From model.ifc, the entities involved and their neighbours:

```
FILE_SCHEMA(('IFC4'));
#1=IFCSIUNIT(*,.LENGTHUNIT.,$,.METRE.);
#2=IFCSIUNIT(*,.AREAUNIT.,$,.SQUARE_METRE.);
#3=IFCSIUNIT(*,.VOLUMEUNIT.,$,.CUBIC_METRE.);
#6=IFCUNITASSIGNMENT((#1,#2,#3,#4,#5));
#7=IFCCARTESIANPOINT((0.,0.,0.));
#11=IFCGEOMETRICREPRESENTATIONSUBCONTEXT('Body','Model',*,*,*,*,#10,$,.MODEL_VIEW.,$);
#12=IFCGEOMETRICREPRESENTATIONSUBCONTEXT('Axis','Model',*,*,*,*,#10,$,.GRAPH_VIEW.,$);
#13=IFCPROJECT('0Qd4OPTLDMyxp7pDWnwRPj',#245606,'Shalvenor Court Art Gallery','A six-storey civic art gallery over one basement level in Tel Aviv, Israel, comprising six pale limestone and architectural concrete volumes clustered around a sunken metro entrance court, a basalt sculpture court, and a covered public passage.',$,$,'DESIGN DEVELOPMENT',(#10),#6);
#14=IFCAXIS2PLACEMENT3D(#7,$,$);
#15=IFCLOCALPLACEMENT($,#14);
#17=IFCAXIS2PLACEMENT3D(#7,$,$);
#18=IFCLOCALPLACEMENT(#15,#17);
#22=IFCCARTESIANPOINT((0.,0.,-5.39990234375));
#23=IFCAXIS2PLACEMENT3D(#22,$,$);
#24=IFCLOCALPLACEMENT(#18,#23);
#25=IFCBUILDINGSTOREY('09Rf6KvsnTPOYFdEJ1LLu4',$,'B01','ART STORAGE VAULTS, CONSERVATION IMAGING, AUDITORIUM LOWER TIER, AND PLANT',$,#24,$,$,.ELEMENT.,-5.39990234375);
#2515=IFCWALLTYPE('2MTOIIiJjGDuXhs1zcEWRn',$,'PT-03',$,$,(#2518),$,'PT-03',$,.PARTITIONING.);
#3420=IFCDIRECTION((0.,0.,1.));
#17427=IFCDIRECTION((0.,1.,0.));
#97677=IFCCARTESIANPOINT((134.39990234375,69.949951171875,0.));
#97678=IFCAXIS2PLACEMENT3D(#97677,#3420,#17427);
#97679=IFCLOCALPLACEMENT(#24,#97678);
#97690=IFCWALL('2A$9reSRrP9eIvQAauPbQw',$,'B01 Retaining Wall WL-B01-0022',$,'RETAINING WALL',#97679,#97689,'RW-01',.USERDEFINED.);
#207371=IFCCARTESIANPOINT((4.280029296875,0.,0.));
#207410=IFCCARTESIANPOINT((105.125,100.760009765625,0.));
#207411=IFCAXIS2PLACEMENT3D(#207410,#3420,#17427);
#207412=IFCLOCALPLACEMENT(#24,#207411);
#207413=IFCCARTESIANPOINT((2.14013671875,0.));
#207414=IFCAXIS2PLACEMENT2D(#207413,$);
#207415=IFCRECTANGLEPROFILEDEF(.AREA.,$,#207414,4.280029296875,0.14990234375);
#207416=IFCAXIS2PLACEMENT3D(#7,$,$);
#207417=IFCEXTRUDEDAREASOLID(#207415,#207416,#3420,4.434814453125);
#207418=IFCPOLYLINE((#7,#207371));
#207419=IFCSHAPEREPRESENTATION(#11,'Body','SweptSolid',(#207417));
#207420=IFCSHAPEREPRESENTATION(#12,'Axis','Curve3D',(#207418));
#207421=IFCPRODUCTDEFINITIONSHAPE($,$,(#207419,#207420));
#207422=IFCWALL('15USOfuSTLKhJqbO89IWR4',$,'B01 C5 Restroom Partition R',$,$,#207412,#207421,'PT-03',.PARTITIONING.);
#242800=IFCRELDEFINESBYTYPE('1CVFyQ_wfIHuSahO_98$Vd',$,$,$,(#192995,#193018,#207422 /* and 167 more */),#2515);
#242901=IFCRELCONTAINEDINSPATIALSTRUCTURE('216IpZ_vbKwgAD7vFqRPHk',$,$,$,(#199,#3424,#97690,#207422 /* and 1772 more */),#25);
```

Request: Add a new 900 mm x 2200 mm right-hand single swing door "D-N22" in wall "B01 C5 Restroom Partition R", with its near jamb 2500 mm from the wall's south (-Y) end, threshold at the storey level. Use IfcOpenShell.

```python
import numpy as np
import ifcopenshell
import ifcopenshell.api.feature
import ifcopenshell.api.geometry
import ifcopenshell.api.root
import ifcopenshell.api.spatial
import ifcopenshell.geom
import ifcopenshell.util.element
import ifcopenshell.util.placement
import ifcopenshell.util.representation
import ifcopenshell.util.shape
import ifcopenshell.util.unit

model = ifcopenshell.open("model.ifc")
unit_scale = ifcopenshell.util.unit.calculate_unit_scale(model)
settings = ifcopenshell.geom.settings()


def volume(element):
    """Net volume in cubic metres, openings subtracted."""
    shape = ifcopenshell.geom.create_shape(settings, element)
    return ifcopenshell.util.shape.get_volume(shape.geometry)


wall = model.by_guid("15USOfuSTLKhJqbO89IWR4")
storey = ifcopenshell.util.element.get_container(wall, ifc_class="IfcBuildingStorey")
context = ifcopenshell.util.representation.get_context(model, "Model", "Body", "MODEL_VIEW")
before = volume(wall)

width, height, from_end, sill = 0.9, 2.2, 2.5, 0.0  # metres

# The wall runs along its own X axis, and the end named is its -X end.
wall_shape = ifcopenshell.geom.create_shape(settings, wall)
x, y, z = ifcopenshell.util.shape.get_vertices(wall_shape.geometry).T
start = x.min() + from_end
face, thickness = float(y.min()), float(y.max() - y.min())
wall_matrix = ifcopenshell.util.placement.get_local_placement(wall.ObjectPlacement)
level = ifcopenshell.util.placement.get_local_placement(storey.ObjectPlacement)[2, 3]


def in_wall(x, y):
    """Placement at x, y metres in the wall's axes, at sill height."""
    matrix = wall_matrix.copy()
    matrix[:, 3] = wall_matrix @ np.array([x / unit_scale, y / unit_scale, 0.0, 1.0])
    matrix[2, 3] = level + sill / unit_scale
    return matrix


# Opening: a box that overshoots both wall faces by 50 mm.
opening = ifcopenshell.api.root.create_entity(model, ifc_class="IfcOpeningElement", predefined_type="OPENING")
box = ifcopenshell.api.geometry.add_wall_representation(
    model, context=context, length=width, height=height, thickness=thickness + 0.1
)
ifcopenshell.api.geometry.assign_representation(model, product=opening, representation=box)
ifcopenshell.api.geometry.edit_object_placement(model, product=opening, matrix=in_wall(start, face - 0.05), is_si=False)
ifcopenshell.api.feature.add_feature(model, feature=opening, element=wall)

door = ifcopenshell.api.root.create_entity(model, ifc_class="IfcDoor", name="D-N22", predefined_type="DOOR")
door.OverallWidth, door.OverallHeight = width / unit_scale, height / unit_scale
door.OperationType = "SINGLE_SWING_RIGHT"
body = ifcopenshell.api.geometry.add_door_representation(
    model,
    context=context,
    overall_width=door.OverallWidth,
    overall_height=door.OverallHeight,
    operation_type="SINGLE_SWING_RIGHT",
    lining_properties={"LiningDepth": thickness / unit_scale, "ThresholdDepth": thickness / unit_scale},
)
ifcopenshell.api.geometry.assign_representation(model, product=door, representation=body)
ifcopenshell.api.spatial.assign_container(model, products=[door], relating_structure=storey)
ifcopenshell.api.feature.add_filling(model, opening=opening, element=door)

# The lining spans the wall, so the door starts at the wall face.
ifcopenshell.api.geometry.edit_object_placement(model, product=door, matrix=in_wall(start, face), is_si=False)

after = volume(wall)

print(f"wall volume {before:.3f} -> {after:.3f} m3")

model.write("model_rev.ifc")
```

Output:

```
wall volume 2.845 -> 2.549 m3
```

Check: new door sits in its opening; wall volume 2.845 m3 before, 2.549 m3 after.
